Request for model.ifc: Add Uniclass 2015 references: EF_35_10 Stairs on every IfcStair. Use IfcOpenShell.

First a look at what the model holds.

```python
import ifcopenshell

model = ifcopenshell.open("model.ifc")
print(model.schema)
print("classifications:", [c.Name for c in model.by_type("IfcClassification")])
for ifc_class in ("IfcDoor", "IfcRoof", "IfcStair", "IfcWall", "IfcWindow"):
    print(ifc_class, len(model.by_type(ifc_class)))
```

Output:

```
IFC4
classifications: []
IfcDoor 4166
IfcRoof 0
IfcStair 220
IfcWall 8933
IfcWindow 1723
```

```python
import ifcopenshell
import ifcopenshell.api.classification

model = ifcopenshell.open("model.ifc")

system = ifcopenshell.api.classification.add_classification(model, classification="Uniclass 2015")

codes = {
    "IfcStair": ("EF_35_10", "Stairs"),
}
for ifc_class, (code, name) in codes.items():
    products = model.by_type(ifc_class)
    ifcopenshell.api.classification.add_reference(
        model, products=products, classification=system, identification=code, name=name
    )
    print(code, len(products))

model.write("model_v2.ifc")
```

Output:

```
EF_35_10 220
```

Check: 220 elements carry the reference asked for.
